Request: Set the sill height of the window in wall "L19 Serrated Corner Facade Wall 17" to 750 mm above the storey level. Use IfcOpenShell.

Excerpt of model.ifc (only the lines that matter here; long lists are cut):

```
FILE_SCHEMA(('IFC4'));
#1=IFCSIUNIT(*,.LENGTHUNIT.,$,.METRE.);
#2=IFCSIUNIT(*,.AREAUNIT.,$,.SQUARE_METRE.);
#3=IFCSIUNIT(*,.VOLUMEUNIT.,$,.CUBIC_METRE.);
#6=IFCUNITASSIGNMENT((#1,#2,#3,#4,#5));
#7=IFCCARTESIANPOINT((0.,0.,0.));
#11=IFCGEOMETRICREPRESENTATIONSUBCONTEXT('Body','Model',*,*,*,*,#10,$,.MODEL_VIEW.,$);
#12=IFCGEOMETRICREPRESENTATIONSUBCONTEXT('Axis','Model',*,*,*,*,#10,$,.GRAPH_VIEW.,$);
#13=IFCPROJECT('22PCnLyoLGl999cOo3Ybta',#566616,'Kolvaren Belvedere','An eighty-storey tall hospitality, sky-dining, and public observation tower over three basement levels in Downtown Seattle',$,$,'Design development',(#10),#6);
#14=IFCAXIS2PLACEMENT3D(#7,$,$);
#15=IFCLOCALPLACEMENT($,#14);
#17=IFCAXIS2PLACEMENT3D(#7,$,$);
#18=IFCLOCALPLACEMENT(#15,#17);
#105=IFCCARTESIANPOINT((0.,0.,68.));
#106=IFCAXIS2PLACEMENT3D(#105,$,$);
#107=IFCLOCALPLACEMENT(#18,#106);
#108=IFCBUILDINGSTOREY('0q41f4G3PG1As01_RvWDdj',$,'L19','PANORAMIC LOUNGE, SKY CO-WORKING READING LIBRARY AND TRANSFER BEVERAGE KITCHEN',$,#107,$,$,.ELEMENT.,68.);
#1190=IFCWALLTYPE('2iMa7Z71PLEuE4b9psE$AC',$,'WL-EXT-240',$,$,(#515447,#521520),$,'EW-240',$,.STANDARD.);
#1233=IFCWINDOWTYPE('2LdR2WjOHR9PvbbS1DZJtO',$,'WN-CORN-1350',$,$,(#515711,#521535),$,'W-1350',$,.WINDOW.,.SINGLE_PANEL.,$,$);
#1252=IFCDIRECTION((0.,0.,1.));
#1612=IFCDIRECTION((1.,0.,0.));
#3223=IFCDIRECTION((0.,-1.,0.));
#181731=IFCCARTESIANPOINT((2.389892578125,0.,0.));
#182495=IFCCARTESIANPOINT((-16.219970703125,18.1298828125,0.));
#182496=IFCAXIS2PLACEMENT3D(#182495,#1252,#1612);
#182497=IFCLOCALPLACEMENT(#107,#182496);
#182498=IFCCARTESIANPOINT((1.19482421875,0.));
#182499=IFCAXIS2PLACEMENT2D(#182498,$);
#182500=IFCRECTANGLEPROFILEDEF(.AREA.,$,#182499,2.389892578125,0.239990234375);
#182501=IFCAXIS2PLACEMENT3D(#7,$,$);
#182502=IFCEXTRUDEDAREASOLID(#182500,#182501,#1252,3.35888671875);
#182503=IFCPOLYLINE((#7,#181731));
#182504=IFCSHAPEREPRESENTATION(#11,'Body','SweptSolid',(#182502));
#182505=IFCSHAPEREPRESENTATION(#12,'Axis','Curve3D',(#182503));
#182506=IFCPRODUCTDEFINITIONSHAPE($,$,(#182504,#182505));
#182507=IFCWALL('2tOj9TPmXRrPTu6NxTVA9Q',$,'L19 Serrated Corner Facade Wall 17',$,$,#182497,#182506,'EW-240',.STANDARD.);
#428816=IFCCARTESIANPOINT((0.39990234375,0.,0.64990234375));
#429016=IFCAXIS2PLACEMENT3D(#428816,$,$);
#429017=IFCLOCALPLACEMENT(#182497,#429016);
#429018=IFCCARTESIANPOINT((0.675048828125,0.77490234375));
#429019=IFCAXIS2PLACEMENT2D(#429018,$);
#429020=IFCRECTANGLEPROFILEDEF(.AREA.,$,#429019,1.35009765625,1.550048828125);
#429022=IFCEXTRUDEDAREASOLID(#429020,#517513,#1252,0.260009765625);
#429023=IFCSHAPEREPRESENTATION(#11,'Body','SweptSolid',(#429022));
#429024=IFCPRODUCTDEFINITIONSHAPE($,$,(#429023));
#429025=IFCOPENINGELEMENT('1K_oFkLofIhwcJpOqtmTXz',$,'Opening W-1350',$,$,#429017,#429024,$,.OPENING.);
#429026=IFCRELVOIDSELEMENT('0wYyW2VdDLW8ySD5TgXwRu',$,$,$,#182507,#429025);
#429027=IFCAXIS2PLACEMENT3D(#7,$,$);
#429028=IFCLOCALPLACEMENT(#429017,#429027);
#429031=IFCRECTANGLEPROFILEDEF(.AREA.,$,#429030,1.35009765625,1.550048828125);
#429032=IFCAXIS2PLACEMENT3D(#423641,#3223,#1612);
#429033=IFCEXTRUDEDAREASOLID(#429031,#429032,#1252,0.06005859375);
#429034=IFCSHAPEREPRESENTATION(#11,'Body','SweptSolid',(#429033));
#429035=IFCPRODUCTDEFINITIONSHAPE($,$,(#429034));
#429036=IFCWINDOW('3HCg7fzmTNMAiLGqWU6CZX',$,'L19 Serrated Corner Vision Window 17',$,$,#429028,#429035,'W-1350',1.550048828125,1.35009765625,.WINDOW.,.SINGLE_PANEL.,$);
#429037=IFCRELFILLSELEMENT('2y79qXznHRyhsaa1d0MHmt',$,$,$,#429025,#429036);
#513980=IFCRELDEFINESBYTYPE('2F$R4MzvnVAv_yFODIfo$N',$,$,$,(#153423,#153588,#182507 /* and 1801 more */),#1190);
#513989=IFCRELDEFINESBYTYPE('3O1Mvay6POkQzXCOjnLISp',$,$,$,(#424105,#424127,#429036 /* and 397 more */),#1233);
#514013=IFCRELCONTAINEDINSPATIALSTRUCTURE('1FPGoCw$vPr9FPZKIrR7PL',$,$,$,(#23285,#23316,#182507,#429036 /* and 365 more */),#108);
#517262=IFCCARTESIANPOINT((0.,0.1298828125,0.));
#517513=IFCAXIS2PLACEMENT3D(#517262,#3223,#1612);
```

```python
import numpy as np
import ifcopenshell
import ifcopenshell.api.geometry
import ifcopenshell.geom
import ifcopenshell.util.element
import ifcopenshell.util.placement
import ifcopenshell.util.shape
import ifcopenshell.util.unit

model = ifcopenshell.open("model.ifc")
unit_scale = ifcopenshell.util.unit.calculate_unit_scale(model)

window = model.by_guid("3HCg7fzmTNMAiLGqWU6CZX")
opening = window.FillsVoids[0].RelatingOpeningElement
storey = ifcopenshell.util.element.get_container(window, ifc_class="IfcBuildingStorey")
level = ifcopenshell.util.placement.get_local_placement(storey.ObjectPlacement)[2, 3]

# The opening's origin need not be at the sill, so measure its lowest point.
shape = ifcopenshell.geom.create_shape(ifcopenshell.geom.settings(), opening)
bottom = ifcopenshell.util.shape.get_shape_bottom_elevation(shape, shape.geometry) / unit_scale
dz = level + 0.75 / unit_scale - bottom

shift = np.array([0.0, 0.0, dz])
# The window is placed relative to its opening, so it follows when the opening moves.
matrix = ifcopenshell.util.placement.get_local_placement(opening.ObjectPlacement)
matrix[:3, 3] += shift
ifcopenshell.api.geometry.edit_object_placement(
    model, product=opening, matrix=matrix, is_si=False, should_transform_children=True
)

print(f"moved by {dz * unit_scale:+.3f} m")

model.write("model_v2.ifc")
```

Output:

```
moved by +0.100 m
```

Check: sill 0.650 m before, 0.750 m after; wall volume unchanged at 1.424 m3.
